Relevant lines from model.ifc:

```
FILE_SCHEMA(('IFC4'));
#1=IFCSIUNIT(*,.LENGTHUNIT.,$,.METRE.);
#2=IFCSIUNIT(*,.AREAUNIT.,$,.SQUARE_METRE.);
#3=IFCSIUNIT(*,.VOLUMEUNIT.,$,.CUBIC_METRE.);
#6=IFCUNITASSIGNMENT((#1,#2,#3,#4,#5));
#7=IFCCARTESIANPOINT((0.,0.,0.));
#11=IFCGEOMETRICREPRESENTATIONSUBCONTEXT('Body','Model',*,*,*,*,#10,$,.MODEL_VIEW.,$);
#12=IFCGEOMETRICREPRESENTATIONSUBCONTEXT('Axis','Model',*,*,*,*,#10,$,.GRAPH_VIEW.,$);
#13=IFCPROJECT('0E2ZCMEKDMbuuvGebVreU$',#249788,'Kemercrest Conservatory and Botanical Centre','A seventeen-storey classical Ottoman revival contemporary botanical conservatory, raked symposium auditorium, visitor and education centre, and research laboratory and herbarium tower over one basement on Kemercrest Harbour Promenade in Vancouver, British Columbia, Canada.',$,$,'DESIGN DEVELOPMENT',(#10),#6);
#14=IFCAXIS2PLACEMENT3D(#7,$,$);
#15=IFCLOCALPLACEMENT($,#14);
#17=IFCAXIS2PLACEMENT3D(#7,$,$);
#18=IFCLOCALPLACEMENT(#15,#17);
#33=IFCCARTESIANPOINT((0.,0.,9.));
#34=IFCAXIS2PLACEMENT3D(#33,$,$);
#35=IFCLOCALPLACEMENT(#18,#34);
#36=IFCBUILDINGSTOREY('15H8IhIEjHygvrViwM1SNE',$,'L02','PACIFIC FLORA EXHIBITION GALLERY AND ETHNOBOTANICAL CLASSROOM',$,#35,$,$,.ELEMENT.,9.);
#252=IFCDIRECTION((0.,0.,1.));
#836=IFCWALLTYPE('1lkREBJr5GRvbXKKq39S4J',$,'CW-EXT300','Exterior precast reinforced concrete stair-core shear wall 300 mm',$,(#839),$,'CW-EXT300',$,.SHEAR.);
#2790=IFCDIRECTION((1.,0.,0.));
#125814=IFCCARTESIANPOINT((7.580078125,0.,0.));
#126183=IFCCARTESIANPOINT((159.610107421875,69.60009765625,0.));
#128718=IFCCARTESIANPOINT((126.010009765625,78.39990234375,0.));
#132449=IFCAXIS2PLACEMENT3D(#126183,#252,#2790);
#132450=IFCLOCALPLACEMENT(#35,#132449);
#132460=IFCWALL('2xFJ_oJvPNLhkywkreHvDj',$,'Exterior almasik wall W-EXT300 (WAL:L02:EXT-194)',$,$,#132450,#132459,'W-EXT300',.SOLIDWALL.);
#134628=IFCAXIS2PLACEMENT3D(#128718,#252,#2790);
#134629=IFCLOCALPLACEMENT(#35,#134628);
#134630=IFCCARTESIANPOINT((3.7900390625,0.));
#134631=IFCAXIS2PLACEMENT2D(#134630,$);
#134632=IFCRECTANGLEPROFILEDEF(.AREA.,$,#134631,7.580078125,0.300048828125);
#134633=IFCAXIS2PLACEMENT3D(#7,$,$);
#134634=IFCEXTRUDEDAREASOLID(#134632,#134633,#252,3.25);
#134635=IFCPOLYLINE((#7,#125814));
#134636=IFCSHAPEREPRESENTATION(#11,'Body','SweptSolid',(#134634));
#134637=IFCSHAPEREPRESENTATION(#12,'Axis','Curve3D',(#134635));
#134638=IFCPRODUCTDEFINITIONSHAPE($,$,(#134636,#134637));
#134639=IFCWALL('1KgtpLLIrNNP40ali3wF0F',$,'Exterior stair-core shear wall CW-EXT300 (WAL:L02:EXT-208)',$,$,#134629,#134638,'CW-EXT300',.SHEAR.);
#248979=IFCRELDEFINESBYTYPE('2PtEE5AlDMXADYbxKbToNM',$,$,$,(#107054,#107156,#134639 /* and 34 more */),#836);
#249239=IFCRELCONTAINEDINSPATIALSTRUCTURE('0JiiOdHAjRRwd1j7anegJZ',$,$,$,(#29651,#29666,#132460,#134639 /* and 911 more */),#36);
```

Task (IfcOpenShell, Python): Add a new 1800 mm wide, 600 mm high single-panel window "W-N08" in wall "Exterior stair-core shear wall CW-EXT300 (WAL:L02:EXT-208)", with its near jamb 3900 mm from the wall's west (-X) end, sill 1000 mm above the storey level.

```python
import numpy as np
import ifcopenshell
import ifcopenshell.api.feature
import ifcopenshell.api.geometry
import ifcopenshell.api.root
import ifcopenshell.api.spatial
import ifcopenshell.geom
import ifcopenshell.util.element
import ifcopenshell.util.placement
import ifcopenshell.util.representation
import ifcopenshell.util.shape
import ifcopenshell.util.unit

model = ifcopenshell.open("model.ifc")
unit_scale = ifcopenshell.util.unit.calculate_unit_scale(model)
settings = ifcopenshell.geom.settings()


def volume(element):
    """Net volume in cubic metres, openings subtracted."""
    shape = ifcopenshell.geom.create_shape(settings, element)
    return ifcopenshell.util.shape.get_volume(shape.geometry)


wall = model.by_guid("1KgtpLLIrNNP40ali3wF0F")
storey = ifcopenshell.util.element.get_container(wall, ifc_class="IfcBuildingStorey")
context = ifcopenshell.util.representation.get_context(model, "Model", "Body", "MODEL_VIEW")
before = volume(wall)

width, height, from_end, sill = 1.8, 0.6, 3.9, 1  # metres

# The wall runs along its own X axis, and the end named is its -X end.
wall_shape = ifcopenshell.geom.create_shape(settings, wall)
x, y, z = ifcopenshell.util.shape.get_vertices(wall_shape.geometry).T
start = x.min() + from_end
face, thickness = float(y.min()), float(y.max() - y.min())
wall_matrix = ifcopenshell.util.placement.get_local_placement(wall.ObjectPlacement)
level = ifcopenshell.util.placement.get_local_placement(storey.ObjectPlacement)[2, 3]


def in_wall(x, y):
    """Placement at x, y metres in the wall's axes, at sill height."""
    matrix = wall_matrix.copy()
    matrix[:, 3] = wall_matrix @ np.array([x / unit_scale, y / unit_scale, 0.0, 1.0])
    matrix[2, 3] = level + sill / unit_scale
    return matrix


# Opening: a box that overshoots both wall faces by 50 mm.
opening = ifcopenshell.api.root.create_entity(model, ifc_class="IfcOpeningElement", predefined_type="OPENING")
box = ifcopenshell.api.geometry.add_wall_representation(
    model, context=context, length=width, height=height, thickness=thickness + 0.1
)
ifcopenshell.api.geometry.assign_representation(model, product=opening, representation=box)
ifcopenshell.api.geometry.edit_object_placement(model, product=opening, matrix=in_wall(start, face - 0.05), is_si=False)
ifcopenshell.api.feature.add_feature(model, feature=opening, element=wall)

window = ifcopenshell.api.root.create_entity(model, ifc_class="IfcWindow", name="W-N08", predefined_type="WINDOW")
window.OverallWidth, window.OverallHeight = width / unit_scale, height / unit_scale
window.PartitioningType = "SINGLE_PANEL"
body = ifcopenshell.api.geometry.add_window_representation(
    model,
    context=context,
    overall_width=window.OverallWidth,
    overall_height=window.OverallHeight,
    partition_type="SINGLE_PANEL",
)
ifcopenshell.api.geometry.assign_representation(model, product=window, representation=body)
ifcopenshell.api.spatial.assign_container(model, products=[window], relating_structure=storey)
ifcopenshell.api.feature.add_filling(model, opening=opening, element=window)

# Centre the window in the wall's thickness.
ifcopenshell.api.geometry.edit_object_placement(model, product=window, matrix=in_wall(start, face), is_si=False)
window_shape = ifcopenshell.geom.create_shape(settings, window)
depth = ifcopenshell.util.shape.get_vertices(window_shape.geometry)[:, 1]
offset = face + thickness / 2 - (depth.min() + depth.max()) / 2
ifcopenshell.api.geometry.edit_object_placement(model, product=window, matrix=in_wall(start, offset), is_si=False)

after = volume(wall)

print(f"wall volume {before:.3f} -> {after:.3f} m3")

model.write("model-out.ifc")
```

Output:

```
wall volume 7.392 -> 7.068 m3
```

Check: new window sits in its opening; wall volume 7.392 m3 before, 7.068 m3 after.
